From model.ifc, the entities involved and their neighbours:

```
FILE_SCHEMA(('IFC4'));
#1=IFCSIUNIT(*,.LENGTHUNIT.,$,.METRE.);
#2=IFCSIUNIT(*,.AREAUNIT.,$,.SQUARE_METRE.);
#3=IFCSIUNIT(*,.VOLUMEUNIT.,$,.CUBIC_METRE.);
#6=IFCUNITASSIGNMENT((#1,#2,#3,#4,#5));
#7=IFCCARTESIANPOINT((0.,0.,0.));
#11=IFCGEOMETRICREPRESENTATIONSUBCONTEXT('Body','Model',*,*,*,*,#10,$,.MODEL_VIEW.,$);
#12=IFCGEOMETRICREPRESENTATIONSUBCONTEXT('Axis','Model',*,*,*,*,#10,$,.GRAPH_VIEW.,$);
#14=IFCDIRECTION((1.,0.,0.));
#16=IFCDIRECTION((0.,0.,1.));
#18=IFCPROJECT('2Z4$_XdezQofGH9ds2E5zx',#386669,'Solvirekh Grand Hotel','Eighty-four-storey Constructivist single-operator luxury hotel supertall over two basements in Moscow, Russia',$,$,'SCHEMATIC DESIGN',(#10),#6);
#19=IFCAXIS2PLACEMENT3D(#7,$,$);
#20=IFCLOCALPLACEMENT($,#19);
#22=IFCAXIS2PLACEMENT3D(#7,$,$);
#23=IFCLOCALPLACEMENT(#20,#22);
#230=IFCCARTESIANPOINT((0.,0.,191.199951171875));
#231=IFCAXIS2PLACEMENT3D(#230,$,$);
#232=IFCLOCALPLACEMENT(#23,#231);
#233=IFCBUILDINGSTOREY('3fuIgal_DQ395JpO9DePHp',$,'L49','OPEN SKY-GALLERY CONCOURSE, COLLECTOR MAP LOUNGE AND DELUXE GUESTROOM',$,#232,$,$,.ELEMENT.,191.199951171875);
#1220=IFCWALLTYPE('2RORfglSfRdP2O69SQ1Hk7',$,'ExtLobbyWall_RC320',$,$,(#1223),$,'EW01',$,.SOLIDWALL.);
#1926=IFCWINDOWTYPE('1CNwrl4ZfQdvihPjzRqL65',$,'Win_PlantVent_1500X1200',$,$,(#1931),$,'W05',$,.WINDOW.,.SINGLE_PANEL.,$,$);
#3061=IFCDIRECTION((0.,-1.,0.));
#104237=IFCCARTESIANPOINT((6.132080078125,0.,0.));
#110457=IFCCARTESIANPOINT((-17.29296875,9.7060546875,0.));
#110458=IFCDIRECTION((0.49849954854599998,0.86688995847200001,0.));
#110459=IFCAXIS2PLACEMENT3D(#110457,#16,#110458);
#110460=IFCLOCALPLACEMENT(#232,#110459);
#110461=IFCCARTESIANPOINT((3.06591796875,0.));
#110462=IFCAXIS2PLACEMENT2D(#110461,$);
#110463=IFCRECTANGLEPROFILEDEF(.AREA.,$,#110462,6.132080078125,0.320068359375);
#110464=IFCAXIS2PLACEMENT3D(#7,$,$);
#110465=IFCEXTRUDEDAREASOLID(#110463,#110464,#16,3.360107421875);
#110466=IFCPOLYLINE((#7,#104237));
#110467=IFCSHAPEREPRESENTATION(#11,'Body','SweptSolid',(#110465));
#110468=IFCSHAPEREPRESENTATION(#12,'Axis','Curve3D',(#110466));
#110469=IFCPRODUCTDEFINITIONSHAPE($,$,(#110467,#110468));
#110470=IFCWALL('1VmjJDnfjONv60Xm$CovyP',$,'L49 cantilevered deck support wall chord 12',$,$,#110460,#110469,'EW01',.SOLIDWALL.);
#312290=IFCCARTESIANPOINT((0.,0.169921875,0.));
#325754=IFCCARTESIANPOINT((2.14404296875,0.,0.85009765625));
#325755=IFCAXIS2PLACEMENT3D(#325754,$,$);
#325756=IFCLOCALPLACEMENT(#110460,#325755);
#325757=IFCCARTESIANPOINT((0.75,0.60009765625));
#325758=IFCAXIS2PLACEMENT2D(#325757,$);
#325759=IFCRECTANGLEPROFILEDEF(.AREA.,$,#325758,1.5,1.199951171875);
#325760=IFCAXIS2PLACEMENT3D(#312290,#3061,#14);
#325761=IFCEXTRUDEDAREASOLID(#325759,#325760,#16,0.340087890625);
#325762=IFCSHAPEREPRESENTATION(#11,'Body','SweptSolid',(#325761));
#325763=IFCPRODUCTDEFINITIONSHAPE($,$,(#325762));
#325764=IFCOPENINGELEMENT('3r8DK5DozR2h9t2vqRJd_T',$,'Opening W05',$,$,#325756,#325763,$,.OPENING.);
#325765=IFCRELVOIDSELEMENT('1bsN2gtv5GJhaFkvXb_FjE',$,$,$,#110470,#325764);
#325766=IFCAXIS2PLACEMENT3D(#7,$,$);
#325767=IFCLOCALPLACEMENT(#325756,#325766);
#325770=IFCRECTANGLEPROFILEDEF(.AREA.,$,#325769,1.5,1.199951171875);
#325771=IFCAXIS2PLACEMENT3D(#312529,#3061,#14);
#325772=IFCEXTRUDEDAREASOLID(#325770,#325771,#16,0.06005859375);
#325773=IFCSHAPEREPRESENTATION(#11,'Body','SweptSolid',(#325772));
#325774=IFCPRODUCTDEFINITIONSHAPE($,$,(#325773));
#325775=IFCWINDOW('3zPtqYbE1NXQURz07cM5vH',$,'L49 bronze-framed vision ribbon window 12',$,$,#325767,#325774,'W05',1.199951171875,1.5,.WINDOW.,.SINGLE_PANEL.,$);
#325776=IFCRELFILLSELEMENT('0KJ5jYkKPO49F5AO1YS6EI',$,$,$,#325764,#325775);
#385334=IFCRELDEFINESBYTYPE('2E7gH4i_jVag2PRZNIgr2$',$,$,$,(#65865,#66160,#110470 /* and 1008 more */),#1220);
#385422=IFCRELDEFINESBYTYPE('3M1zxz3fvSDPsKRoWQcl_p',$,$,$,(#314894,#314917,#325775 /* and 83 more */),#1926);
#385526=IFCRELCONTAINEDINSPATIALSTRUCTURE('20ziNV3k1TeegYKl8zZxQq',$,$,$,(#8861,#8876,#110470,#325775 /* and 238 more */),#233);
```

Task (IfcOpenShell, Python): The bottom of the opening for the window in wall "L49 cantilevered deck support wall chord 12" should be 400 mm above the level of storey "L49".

```python
import numpy as np
import ifcopenshell
import ifcopenshell.api.geometry
import ifcopenshell.geom
import ifcopenshell.util.element
import ifcopenshell.util.placement
import ifcopenshell.util.shape
import ifcopenshell.util.unit

model = ifcopenshell.open("model.ifc")
unit_scale = ifcopenshell.util.unit.calculate_unit_scale(model)

window = model.by_guid("3zPtqYbE1NXQURz07cM5vH")
opening = window.FillsVoids[0].RelatingOpeningElement
storey = ifcopenshell.util.element.get_container(window, ifc_class="IfcBuildingStorey")
level = ifcopenshell.util.placement.get_local_placement(storey.ObjectPlacement)[2, 3]

# The opening's origin need not be at the sill, so measure its lowest point.
shape = ifcopenshell.geom.create_shape(ifcopenshell.geom.settings(), opening)
bottom = ifcopenshell.util.shape.get_shape_bottom_elevation(shape, shape.geometry) / unit_scale
dz = level + 0.4 / unit_scale - bottom

shift = np.array([0.0, 0.0, dz])
# The window is placed relative to its opening, so it follows when the opening moves.
matrix = ifcopenshell.util.placement.get_local_placement(opening.ObjectPlacement)
matrix[:3, 3] += shift
ifcopenshell.api.geometry.edit_object_placement(
    model, product=opening, matrix=matrix, is_si=False, should_transform_children=True
)

print(f"moved by {dz * unit_scale:+.3f} m")

model.write("model_v2.ifc")
```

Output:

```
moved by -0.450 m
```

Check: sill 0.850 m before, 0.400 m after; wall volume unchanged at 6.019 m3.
